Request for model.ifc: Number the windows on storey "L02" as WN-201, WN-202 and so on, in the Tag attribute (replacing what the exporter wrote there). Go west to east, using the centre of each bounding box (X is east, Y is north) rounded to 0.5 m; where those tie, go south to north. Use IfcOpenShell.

First a look at what the model holds.

```python
import ifcopenshell
import ifcopenshell.util.element
import ifcopenshell.util.placement

model = ifcopenshell.open("model.ifc")
print(model.schema)
storey = next(s for s in model.by_type("IfcBuildingStorey") if s.Name == "L02")
windows = [e for e in ifcopenshell.util.element.get_decomposition(storey) if e.is_a("IfcWindow")]
for e in sorted(windows, key=lambda e: e.id()):
    origin = ifcopenshell.util.placement.get_local_placement(e.ObjectPlacement)[:3, 3]
    print(e.id(), e.Tag, e.Name, origin.round(2) + 0.0, sep=" | ")
```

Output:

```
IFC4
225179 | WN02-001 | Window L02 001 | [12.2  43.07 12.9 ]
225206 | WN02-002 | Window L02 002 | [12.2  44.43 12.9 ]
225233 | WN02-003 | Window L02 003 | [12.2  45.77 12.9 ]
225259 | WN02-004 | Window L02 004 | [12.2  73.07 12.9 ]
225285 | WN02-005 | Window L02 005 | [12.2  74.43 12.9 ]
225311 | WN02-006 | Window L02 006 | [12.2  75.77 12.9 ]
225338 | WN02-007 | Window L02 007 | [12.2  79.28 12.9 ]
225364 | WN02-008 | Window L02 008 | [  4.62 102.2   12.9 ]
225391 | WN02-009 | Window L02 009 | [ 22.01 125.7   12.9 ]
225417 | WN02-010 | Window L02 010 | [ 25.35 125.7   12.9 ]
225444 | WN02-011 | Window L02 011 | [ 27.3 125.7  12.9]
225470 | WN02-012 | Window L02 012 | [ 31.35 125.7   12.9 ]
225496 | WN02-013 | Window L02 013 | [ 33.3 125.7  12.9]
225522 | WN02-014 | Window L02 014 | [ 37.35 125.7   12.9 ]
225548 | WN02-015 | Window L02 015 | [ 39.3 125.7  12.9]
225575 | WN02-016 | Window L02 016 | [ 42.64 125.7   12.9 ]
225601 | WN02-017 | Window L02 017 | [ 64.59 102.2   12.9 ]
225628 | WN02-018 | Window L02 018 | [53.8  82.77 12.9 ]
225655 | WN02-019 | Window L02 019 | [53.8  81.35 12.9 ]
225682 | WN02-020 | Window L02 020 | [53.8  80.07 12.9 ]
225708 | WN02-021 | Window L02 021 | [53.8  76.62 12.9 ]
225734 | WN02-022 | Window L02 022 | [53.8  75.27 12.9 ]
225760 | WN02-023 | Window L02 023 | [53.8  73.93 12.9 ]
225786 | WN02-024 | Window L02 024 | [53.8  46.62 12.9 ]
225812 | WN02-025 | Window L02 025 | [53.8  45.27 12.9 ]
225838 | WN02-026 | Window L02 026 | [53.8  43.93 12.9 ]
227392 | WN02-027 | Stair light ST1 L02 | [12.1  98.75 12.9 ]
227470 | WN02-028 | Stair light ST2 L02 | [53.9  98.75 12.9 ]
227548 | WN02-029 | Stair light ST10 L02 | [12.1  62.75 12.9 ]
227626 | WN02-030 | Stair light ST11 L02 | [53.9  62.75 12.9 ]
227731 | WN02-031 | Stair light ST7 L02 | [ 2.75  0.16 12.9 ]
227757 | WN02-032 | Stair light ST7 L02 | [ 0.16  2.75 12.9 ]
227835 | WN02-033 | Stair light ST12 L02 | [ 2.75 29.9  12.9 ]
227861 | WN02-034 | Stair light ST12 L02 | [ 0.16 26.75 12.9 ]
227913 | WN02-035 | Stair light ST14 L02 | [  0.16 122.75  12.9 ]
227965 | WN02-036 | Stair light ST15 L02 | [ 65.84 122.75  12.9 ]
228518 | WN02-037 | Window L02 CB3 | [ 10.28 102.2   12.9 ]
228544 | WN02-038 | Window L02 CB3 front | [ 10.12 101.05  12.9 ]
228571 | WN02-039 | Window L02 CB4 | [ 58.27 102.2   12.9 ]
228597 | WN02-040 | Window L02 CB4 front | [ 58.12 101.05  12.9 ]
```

```python
import ifcopenshell
import ifcopenshell.geom
import ifcopenshell.util.element
import ifcopenshell.util.shape

model = ifcopenshell.open("model.ifc")
settings = ifcopenshell.geom.settings()
settings.set("use-world-coords", True)


def centre(element):
    shape = ifcopenshell.geom.create_shape(settings, element)
    return ifcopenshell.util.shape.get_bbox_centroid(shape.geometry)


storey = next(s for s in model.by_type("IfcBuildingStorey") if s.Name == "L02")
windows = [e for e in ifcopenshell.util.element.get_decomposition(storey) if e.is_a("IfcWindow")]

# Insertion points can sit at a corner or the storey origin, so sort by the geometry (in metres).
centres = {e: centre(e) for e in windows}
windows.sort(key=lambda e: (round(centres[e][0] / 0.5), centres[e][1]))

for i, e in enumerate(windows, start=1):
    number = f"WN-2{i:02d}"
    e.Tag = number
    print(e.id(), number)

model.write("model-out.ifc")
```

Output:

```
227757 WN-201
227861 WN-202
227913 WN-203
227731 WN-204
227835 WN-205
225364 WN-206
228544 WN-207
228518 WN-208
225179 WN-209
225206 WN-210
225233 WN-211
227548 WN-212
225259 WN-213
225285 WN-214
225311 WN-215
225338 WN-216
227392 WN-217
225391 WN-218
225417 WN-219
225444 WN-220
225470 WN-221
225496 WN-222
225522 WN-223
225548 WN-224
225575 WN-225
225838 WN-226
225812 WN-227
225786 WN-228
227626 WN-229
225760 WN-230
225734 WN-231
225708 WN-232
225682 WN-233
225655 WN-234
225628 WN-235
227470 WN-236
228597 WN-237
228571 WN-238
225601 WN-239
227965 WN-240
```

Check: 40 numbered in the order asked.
